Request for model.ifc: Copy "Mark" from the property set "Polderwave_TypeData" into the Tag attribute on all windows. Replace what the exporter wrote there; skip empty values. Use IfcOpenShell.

First a look at what the model holds.

```python
import ifcopenshell
import ifcopenshell.util.element

model = ifcopenshell.open("model.ifc")
print(model.schema)
windows = model.by_type("IfcWindow")
print(len(windows), "windows")
for e in windows[:8]:
    source = ifcopenshell.util.element.get_pset(e, "Polderwave_TypeData", "Mark")
    target = e.Tag
    print(e.id(), repr(source), repr(target), sep=" | ")
```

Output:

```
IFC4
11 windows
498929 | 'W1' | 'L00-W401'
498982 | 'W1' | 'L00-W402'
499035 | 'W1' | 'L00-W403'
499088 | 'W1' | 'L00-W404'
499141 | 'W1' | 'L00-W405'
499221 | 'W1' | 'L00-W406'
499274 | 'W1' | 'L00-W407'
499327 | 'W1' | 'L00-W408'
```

```python
import ifcopenshell
import ifcopenshell.util.element

model = ifcopenshell.open("model.ifc")

count = 0
for e in model.by_type("IfcWindow"):
    value = ifcopenshell.util.element.get_pset(e, "Polderwave_TypeData", "Mark")
    current = e.Tag
    if not value or not value.strip() or current == value:
        continue
    e.Tag = value
    count += 1

print(count, "windows updated")

model.write("model_edited.ifc")
```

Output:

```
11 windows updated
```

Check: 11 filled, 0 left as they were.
